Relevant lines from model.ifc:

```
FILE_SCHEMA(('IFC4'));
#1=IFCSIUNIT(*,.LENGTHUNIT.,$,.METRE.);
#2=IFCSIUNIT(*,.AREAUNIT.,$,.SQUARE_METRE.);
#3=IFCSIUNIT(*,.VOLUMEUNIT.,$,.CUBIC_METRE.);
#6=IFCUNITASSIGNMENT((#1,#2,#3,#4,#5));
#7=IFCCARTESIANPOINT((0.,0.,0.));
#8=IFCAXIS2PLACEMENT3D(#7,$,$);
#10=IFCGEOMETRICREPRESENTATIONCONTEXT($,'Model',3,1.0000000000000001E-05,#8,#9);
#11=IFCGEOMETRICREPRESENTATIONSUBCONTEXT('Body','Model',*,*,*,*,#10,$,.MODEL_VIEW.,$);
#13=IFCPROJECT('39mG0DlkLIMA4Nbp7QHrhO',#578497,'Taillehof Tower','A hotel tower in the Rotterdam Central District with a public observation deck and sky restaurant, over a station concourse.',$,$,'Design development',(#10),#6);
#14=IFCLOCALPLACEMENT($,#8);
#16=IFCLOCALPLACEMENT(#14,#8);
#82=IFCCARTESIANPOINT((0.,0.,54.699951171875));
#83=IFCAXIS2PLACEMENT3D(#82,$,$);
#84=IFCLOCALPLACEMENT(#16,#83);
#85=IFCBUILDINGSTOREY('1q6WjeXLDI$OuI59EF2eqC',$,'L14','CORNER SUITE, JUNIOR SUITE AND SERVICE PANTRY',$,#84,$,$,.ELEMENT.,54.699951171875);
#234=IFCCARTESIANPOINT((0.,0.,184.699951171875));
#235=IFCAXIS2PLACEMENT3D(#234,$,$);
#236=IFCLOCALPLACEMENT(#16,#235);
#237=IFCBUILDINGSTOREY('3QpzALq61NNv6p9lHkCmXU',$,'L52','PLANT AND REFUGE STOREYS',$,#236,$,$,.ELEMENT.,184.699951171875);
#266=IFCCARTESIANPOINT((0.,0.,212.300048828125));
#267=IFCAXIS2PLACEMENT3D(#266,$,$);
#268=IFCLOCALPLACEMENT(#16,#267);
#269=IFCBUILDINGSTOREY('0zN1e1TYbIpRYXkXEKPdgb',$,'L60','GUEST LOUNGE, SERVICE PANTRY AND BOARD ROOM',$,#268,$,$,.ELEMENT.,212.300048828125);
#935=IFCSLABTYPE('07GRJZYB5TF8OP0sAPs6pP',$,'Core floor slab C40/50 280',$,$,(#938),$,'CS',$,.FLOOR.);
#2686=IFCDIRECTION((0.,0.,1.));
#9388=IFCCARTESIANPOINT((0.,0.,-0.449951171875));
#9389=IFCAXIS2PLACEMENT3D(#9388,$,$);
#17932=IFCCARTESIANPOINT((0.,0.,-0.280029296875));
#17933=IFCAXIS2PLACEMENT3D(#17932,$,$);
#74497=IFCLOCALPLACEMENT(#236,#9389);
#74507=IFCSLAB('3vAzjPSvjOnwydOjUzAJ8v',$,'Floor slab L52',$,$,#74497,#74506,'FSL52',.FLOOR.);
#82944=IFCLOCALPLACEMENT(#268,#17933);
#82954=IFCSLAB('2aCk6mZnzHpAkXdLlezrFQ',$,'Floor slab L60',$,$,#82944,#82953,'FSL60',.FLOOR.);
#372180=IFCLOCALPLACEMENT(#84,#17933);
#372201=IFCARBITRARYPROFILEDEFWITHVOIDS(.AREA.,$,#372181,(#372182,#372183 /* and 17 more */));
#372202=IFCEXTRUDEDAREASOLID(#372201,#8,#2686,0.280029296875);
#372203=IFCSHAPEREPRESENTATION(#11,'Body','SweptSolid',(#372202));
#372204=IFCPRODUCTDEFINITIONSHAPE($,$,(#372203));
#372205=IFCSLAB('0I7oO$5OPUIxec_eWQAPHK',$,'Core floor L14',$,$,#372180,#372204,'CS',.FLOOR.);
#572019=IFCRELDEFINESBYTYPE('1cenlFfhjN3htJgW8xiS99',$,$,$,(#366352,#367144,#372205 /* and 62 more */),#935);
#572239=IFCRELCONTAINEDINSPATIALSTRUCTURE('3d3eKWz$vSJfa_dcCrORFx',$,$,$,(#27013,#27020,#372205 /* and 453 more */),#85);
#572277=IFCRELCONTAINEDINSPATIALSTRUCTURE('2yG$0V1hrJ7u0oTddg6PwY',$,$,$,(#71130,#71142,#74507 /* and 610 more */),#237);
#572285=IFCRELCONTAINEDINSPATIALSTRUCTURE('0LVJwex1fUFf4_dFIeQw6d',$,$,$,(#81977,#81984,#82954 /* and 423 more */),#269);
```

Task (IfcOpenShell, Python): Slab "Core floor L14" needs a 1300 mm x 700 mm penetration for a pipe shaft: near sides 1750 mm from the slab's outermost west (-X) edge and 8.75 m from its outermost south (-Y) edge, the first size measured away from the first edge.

```python
import numpy as np
import ifcopenshell
import ifcopenshell.api.feature
import ifcopenshell.api.geometry
import ifcopenshell.api.root
import ifcopenshell.geom
import ifcopenshell.util.placement
import ifcopenshell.util.representation
import ifcopenshell.util.shape
import ifcopenshell.util.unit

model = ifcopenshell.open("model.ifc")
unit_scale = ifcopenshell.util.unit.calculate_unit_scale(model)
settings = ifcopenshell.geom.settings()


def volume(element):
    """Net volume in cubic metres, openings subtracted."""
    shape = ifcopenshell.geom.create_shape(settings, element)
    return ifcopenshell.util.shape.get_volume(shape.geometry)


slab = model.by_id(372205)
before = volume(slab)

# Extent in the slab's own axes, in metres. The edges named are its -X and -Y sides.
slab_shape = ifcopenshell.geom.create_shape(settings, slab)
vertices = ifcopenshell.util.shape.get_vertices(slab_shape.geometry)
x_min, y_min, bottom = vertices.min(axis=0)
top = vertices[:, 2].max()

opening = ifcopenshell.api.root.create_entity(model, ifc_class="IfcOpeningElement", name="Pipe shaft opening", predefined_type="OPENING")
context = ifcopenshell.util.representation.get_context(model, "Model", "Body", "MODEL_VIEW")
width, depth = 1.3, 0.7
outline = [(0.0, 0.0), (width, 0.0), (width, depth), (0.0, depth), (0.0, 0.0)]
# Overshoot both faces by 50 mm so the cut is clean.
shape = ifcopenshell.api.geometry.add_slab_representation(
    model, context=context, depth=top - bottom + 0.1, polyline=outline
)
ifcopenshell.api.geometry.assign_representation(model, product=opening, representation=shape)

matrix = ifcopenshell.util.placement.get_local_placement(slab.ObjectPlacement)
matrix[:, 3] = matrix @ np.append(np.array([x_min + 1.75, y_min + 8.75, bottom - 0.05]) / unit_scale, 1.0)
ifcopenshell.api.geometry.edit_object_placement(model, product=opening, matrix=matrix, is_si=False)
ifcopenshell.api.feature.add_feature(model, feature=opening, element=slab)

after = volume(slab)

print(f"slab volume {before:.3f} -> {after:.3f} m3")

model.write("model_updated.ifc")
```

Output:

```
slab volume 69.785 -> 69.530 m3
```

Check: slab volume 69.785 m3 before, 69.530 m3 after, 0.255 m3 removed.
